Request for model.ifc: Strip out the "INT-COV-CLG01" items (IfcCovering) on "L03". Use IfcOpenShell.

First a look at what the model holds.

```python
import ifcopenshell
import ifcopenshell.util.element

model = ifcopenshell.open("model.ifc")
print(model.schema)
storey = next(s for s in model.by_type("IfcBuildingStorey") if s.Name == "L03")
coverings = [e for e in ifcopenshell.util.element.get_decomposition(storey) if e.is_a("IfcCovering")]
seen = {}
for e in coverings:
    element_type = ifcopenshell.util.element.get_type(e)
    name = element_type.Name if element_type not in (None, e) else None
    seen[name] = seen.get(name, 0) + 1
for name, count in sorted(seen.items(), key=str):
    print(count, "x", name)
```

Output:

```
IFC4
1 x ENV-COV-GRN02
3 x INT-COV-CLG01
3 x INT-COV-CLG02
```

```python
import ifcopenshell
import ifcopenshell.api.root
import ifcopenshell.util.element

model = ifcopenshell.open("model.ifc")

storey = next(s for s in model.by_type("IfcBuildingStorey") if s.Name == "L03")
coverings = [e for e in ifcopenshell.util.element.get_decomposition(storey) if e.is_a("IfcCovering")]
targets = [e for e in coverings if (t := ifcopenshell.util.element.get_type(e)) not in (None, e) and t.Name == "INT-COV-CLG01"]

for e in targets:
    ifcopenshell.api.root.remove_product(model, product=e)
print(len(targets), "removed")

model.write("model_v2.ifc")
```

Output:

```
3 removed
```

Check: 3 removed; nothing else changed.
